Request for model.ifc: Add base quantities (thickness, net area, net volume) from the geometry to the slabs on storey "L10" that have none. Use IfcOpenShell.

First a look at what the model holds.

```python
import ifcopenshell
import ifcopenshell.util.element
import ifcopenshell.util.unit

model = ifcopenshell.open("model.ifc")
print(model.schema)
for unit_type in ("LENGTHUNIT", "AREAUNIT", "VOLUMEUNIT"):
    print(unit_type, ifcopenshell.util.unit.calculate_unit_scale(model, unit_type))
storey = next(s for s in model.by_type("IfcBuildingStorey") if s.Name == "L10")
slabs = [e for e in ifcopenshell.util.element.get_decomposition(storey) if e.is_a("IfcSlab")]
for e in sorted(slabs, key=lambda e: e.id()):
    print(e.id(), e.is_a(), e.Name, list(ifcopenshell.util.element.get_psets(e, qtos_only=True)), sep=" | ")
```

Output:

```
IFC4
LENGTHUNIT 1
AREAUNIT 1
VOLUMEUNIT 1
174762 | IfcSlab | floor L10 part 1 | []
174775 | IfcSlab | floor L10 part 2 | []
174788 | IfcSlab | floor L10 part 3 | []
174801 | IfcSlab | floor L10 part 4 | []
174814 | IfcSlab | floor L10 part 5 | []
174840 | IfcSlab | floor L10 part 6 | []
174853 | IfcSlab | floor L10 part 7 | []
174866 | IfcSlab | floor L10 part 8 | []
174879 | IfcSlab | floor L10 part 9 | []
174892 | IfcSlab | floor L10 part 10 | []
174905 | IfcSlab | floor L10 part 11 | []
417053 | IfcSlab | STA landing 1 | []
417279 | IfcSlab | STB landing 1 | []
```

```python
import ifcopenshell
import ifcopenshell.api.pset
import ifcopenshell.geom
import ifcopenshell.util.element
import ifcopenshell.util.shape
import ifcopenshell.util.unit

model = ifcopenshell.open("model.ifc")
unit_scale = ifcopenshell.util.unit.calculate_unit_scale(model)
area_scale = ifcopenshell.util.unit.calculate_unit_scale(model, "AREAUNIT")
volume_scale = ifcopenshell.util.unit.calculate_unit_scale(model, "VOLUMEUNIT")
settings = ifcopenshell.geom.settings()

storey = next(s for s in model.by_type("IfcBuildingStorey") if s.Name == "L10")
slabs = [e for e in ifcopenshell.util.element.get_decomposition(storey) if e.is_a("IfcSlab")]

for e in sorted(slabs, key=lambda e: e.id()):
    if ifcopenshell.util.element.get_psets(e, qtos_only=True, should_inherit=False):
        continue
    # Geometry comes back in metres, in the element's own axes.
    shape = ifcopenshell.geom.create_shape(settings, e)
    values = {
        "Width": ifcopenshell.util.shape.get_z(shape.geometry) / unit_scale,
        "NetArea": ifcopenshell.util.shape.get_footprint_area(shape.geometry) / area_scale,
        "NetVolume": ifcopenshell.util.shape.get_volume(shape.geometry) / volume_scale,
    }
    qto = ifcopenshell.api.pset.add_qto(model, product=e, name="Qto_SlabBaseQuantities")
    ifcopenshell.api.pset.edit_qto(model, qto=qto, properties=values)
    print(e.id(), {k: round(v, 3) for k, v in values.items()})

model.write("model_edited.ifc")
```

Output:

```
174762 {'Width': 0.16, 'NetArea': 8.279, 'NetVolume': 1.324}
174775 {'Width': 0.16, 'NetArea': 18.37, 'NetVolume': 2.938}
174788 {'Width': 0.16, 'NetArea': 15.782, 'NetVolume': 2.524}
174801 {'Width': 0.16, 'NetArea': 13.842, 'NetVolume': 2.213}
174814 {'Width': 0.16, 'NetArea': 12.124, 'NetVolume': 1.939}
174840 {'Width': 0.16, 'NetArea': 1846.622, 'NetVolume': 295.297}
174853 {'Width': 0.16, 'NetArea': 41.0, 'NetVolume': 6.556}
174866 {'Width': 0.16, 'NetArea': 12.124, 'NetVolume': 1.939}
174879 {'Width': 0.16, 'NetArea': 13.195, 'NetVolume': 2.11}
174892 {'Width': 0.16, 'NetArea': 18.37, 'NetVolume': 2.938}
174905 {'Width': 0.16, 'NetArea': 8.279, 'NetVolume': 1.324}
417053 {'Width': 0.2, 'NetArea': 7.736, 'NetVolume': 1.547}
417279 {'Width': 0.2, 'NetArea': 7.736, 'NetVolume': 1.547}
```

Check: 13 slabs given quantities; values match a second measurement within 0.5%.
